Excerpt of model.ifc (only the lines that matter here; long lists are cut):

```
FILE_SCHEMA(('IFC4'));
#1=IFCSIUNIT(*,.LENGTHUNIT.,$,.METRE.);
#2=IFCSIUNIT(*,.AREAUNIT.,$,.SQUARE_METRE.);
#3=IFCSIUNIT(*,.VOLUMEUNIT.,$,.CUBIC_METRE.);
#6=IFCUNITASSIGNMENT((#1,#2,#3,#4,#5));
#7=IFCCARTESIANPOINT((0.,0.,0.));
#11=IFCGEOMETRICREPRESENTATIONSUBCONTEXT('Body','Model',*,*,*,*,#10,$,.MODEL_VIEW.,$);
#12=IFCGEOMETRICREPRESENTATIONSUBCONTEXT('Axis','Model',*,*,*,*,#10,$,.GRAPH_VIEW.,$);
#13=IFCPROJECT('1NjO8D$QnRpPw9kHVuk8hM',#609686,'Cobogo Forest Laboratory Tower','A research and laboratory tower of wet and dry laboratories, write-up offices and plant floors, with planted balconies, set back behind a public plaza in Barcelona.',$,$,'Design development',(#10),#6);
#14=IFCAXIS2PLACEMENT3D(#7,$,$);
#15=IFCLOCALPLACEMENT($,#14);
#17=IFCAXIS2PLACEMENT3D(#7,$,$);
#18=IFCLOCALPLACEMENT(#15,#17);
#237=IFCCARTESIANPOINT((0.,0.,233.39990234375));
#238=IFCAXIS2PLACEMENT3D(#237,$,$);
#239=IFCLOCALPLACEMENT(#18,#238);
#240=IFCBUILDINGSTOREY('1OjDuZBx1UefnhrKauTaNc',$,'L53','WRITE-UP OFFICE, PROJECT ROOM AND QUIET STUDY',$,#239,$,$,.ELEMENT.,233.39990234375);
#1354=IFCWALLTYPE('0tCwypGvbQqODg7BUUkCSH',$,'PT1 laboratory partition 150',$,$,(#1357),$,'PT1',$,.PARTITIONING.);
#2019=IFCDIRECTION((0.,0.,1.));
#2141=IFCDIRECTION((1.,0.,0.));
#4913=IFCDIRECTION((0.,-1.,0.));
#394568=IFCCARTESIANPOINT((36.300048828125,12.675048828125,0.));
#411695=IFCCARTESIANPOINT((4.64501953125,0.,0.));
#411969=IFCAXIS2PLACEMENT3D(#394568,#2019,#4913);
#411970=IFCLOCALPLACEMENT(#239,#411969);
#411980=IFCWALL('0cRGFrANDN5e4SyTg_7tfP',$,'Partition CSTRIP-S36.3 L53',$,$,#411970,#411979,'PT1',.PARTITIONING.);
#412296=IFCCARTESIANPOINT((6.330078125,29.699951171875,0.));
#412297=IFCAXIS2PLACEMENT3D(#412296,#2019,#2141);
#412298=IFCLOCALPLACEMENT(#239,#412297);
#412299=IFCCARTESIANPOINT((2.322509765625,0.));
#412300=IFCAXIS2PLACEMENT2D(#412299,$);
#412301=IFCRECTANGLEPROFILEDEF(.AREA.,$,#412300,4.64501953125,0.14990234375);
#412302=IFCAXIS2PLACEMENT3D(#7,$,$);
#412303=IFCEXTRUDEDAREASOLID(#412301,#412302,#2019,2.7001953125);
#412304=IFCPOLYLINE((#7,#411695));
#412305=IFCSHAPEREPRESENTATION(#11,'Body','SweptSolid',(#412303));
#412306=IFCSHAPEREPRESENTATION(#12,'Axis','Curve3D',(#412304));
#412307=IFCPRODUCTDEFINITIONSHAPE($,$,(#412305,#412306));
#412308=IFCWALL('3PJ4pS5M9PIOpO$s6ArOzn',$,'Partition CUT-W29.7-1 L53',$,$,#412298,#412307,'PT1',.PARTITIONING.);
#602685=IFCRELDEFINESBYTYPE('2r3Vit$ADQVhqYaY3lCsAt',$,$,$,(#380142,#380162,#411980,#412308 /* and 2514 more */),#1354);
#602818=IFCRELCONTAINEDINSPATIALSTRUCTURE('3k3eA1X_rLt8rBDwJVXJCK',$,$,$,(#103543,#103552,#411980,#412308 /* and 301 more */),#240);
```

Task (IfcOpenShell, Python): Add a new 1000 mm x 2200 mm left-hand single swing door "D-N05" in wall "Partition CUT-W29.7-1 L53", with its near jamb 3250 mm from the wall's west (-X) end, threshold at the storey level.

```python
import numpy as np
import ifcopenshell
import ifcopenshell.api.feature
import ifcopenshell.api.geometry
import ifcopenshell.api.root
import ifcopenshell.api.spatial
import ifcopenshell.geom
import ifcopenshell.util.element
import ifcopenshell.util.placement
import ifcopenshell.util.representation
import ifcopenshell.util.shape
import ifcopenshell.util.unit

model = ifcopenshell.open("model.ifc")
unit_scale = ifcopenshell.util.unit.calculate_unit_scale(model)
settings = ifcopenshell.geom.settings()


def volume(element):
    """Net volume in cubic metres, openings subtracted."""
    shape = ifcopenshell.geom.create_shape(settings, element)
    return ifcopenshell.util.shape.get_volume(shape.geometry)


wall = model.by_guid("3PJ4pS5M9PIOpO$s6ArOzn")
storey = ifcopenshell.util.element.get_container(wall, ifc_class="IfcBuildingStorey")
context = ifcopenshell.util.representation.get_context(model, "Model", "Body", "MODEL_VIEW")
before = volume(wall)

width, height, from_end, sill = 1, 2.2, 3.25, 0.0  # metres

# The wall runs along its own X axis, and the end named is its -X end.
wall_shape = ifcopenshell.geom.create_shape(settings, wall)
x, y, z = ifcopenshell.util.shape.get_vertices(wall_shape.geometry).T
start = x.min() + from_end
face, thickness = float(y.min()), float(y.max() - y.min())
wall_matrix = ifcopenshell.util.placement.get_local_placement(wall.ObjectPlacement)
level = ifcopenshell.util.placement.get_local_placement(storey.ObjectPlacement)[2, 3]


def in_wall(x, y):
    """Placement at x, y metres in the wall's axes, at sill height."""
    matrix = wall_matrix.copy()
    matrix[:, 3] = wall_matrix @ np.array([x / unit_scale, y / unit_scale, 0.0, 1.0])
    matrix[2, 3] = level + sill / unit_scale
    return matrix


# Opening: a box that overshoots both wall faces by 50 mm.
opening = ifcopenshell.api.root.create_entity(model, ifc_class="IfcOpeningElement", predefined_type="OPENING")
box = ifcopenshell.api.geometry.add_wall_representation(
    model, context=context, length=width, height=height, thickness=thickness + 0.1
)
ifcopenshell.api.geometry.assign_representation(model, product=opening, representation=box)
ifcopenshell.api.geometry.edit_object_placement(model, product=opening, matrix=in_wall(start, face - 0.05), is_si=False)
ifcopenshell.api.feature.add_feature(model, feature=opening, element=wall)

door = ifcopenshell.api.root.create_entity(model, ifc_class="IfcDoor", name="D-N05", predefined_type="DOOR")
door.OverallWidth, door.OverallHeight = width / unit_scale, height / unit_scale
door.OperationType = "SINGLE_SWING_LEFT"
body = ifcopenshell.api.geometry.add_door_representation(
    model,
    context=context,
    overall_width=door.OverallWidth,
    overall_height=door.OverallHeight,
    operation_type="SINGLE_SWING_LEFT",
    lining_properties={"LiningDepth": thickness / unit_scale, "ThresholdDepth": thickness / unit_scale},
)
ifcopenshell.api.geometry.assign_representation(model, product=door, representation=body)
ifcopenshell.api.spatial.assign_container(model, products=[door], relating_structure=storey)
ifcopenshell.api.feature.add_filling(model, opening=opening, element=door)

# The lining spans the wall, so the door starts at the wall face.
ifcopenshell.api.geometry.edit_object_placement(model, product=door, matrix=in_wall(start, face), is_si=False)

after = volume(wall)

print(f"wall volume {before:.3f} -> {after:.3f} m3")

model.write("model_edited.ifc")
```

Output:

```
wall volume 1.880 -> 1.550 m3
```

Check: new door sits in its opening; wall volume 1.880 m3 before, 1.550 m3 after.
